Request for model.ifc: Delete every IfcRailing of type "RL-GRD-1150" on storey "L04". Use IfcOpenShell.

First a look at what the model holds.

```python
import ifcopenshell
import ifcopenshell.util.element

model = ifcopenshell.open("model.ifc")
print(model.schema)
storey = next(s for s in model.by_type("IfcBuildingStorey") if s.Name == "L04")
railings = [e for e in ifcopenshell.util.element.get_decomposition(storey) if e.is_a("IfcRailing")]
seen = {}
for e in railings:
    element_type = ifcopenshell.util.element.get_type(e)
    name = element_type.Name if element_type not in (None, e) else None
    seen[name] = seen.get(name, 0) + 1
for name, count in sorted(seen.items(), key=str):
    print(count, "x", name)
```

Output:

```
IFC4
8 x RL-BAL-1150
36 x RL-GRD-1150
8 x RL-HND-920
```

```python
import ifcopenshell
import ifcopenshell.api.root
import ifcopenshell.util.element

model = ifcopenshell.open("model.ifc")

storey = next(s for s in model.by_type("IfcBuildingStorey") if s.Name == "L04")
railings = [e for e in ifcopenshell.util.element.get_decomposition(storey) if e.is_a("IfcRailing")]
targets = [e for e in railings if (t := ifcopenshell.util.element.get_type(e)) not in (None, e) and t.Name == "RL-GRD-1150"]

for e in targets:
    ifcopenshell.api.root.remove_product(model, product=e)
print(len(targets), "removed")

model.write("model-out.ifc")
```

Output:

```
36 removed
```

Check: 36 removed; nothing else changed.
